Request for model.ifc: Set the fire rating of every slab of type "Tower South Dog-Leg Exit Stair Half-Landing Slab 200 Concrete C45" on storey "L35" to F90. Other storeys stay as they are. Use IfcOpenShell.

First a look at what the model holds.

```python
import ifcopenshell
import ifcopenshell.util.element

model = ifcopenshell.open("model.ifc")
print(model.schema)
storey = next(s for s in model.by_type("IfcBuildingStorey") if s.Name == "L35")
slabs = [e for e in ifcopenshell.util.element.get_decomposition(storey) if e.is_a("IfcSlab")]
seen = {}
for e in slabs:
    element_type = ifcopenshell.util.element.get_type(e)
    key = (element_type.Name if element_type != e and element_type else None, ifcopenshell.util.element.get_pset(e, "Pset_SlabCommon", "FireRating"))
    seen[key] = seen.get(key, 0) + 1
for (name, value), count in sorted(seen.items(), key=str):
    print(count, "x", name, "|", value)
```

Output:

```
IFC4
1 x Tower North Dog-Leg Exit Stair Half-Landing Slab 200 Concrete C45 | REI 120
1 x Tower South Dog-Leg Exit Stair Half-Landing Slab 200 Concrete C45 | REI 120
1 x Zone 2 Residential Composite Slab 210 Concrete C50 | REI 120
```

```python
import ifcopenshell
import ifcopenshell.api.pset
import ifcopenshell.util.element

model = ifcopenshell.open("model.ifc")

storey = next(s for s in model.by_type("IfcBuildingStorey") if s.Name == "L35")
slabs = [e for e in ifcopenshell.util.element.get_decomposition(storey) if e.is_a("IfcSlab")]

count = 0
for e in slabs:
    element_type = ifcopenshell.util.element.get_type(e)
    if element_type in (None, e) or element_type.Name != "Tower South Dog-Leg Exit Stair Half-Landing Slab 200 Concrete C45":
        continue
    found = ifcopenshell.util.element.get_pset(e, "Pset_SlabCommon", should_inherit=False)
    if found:
        pset = model.by_id(found["id"])
        if len(ifcopenshell.util.element.get_elements_by_pset(pset)) > 1:
            pset = ifcopenshell.api.pset.unshare_pset(model, products=[e], pset=pset)[0]
    else:
        pset = ifcopenshell.api.pset.add_pset(model, product=e, name="Pset_SlabCommon")
    ifcopenshell.api.pset.edit_pset(model, pset=pset, properties={"FireRating": "F90"})
    count += 1

print(count, "slabs updated")

model.write("model_v2.ifc")
```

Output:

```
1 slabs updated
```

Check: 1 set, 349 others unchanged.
